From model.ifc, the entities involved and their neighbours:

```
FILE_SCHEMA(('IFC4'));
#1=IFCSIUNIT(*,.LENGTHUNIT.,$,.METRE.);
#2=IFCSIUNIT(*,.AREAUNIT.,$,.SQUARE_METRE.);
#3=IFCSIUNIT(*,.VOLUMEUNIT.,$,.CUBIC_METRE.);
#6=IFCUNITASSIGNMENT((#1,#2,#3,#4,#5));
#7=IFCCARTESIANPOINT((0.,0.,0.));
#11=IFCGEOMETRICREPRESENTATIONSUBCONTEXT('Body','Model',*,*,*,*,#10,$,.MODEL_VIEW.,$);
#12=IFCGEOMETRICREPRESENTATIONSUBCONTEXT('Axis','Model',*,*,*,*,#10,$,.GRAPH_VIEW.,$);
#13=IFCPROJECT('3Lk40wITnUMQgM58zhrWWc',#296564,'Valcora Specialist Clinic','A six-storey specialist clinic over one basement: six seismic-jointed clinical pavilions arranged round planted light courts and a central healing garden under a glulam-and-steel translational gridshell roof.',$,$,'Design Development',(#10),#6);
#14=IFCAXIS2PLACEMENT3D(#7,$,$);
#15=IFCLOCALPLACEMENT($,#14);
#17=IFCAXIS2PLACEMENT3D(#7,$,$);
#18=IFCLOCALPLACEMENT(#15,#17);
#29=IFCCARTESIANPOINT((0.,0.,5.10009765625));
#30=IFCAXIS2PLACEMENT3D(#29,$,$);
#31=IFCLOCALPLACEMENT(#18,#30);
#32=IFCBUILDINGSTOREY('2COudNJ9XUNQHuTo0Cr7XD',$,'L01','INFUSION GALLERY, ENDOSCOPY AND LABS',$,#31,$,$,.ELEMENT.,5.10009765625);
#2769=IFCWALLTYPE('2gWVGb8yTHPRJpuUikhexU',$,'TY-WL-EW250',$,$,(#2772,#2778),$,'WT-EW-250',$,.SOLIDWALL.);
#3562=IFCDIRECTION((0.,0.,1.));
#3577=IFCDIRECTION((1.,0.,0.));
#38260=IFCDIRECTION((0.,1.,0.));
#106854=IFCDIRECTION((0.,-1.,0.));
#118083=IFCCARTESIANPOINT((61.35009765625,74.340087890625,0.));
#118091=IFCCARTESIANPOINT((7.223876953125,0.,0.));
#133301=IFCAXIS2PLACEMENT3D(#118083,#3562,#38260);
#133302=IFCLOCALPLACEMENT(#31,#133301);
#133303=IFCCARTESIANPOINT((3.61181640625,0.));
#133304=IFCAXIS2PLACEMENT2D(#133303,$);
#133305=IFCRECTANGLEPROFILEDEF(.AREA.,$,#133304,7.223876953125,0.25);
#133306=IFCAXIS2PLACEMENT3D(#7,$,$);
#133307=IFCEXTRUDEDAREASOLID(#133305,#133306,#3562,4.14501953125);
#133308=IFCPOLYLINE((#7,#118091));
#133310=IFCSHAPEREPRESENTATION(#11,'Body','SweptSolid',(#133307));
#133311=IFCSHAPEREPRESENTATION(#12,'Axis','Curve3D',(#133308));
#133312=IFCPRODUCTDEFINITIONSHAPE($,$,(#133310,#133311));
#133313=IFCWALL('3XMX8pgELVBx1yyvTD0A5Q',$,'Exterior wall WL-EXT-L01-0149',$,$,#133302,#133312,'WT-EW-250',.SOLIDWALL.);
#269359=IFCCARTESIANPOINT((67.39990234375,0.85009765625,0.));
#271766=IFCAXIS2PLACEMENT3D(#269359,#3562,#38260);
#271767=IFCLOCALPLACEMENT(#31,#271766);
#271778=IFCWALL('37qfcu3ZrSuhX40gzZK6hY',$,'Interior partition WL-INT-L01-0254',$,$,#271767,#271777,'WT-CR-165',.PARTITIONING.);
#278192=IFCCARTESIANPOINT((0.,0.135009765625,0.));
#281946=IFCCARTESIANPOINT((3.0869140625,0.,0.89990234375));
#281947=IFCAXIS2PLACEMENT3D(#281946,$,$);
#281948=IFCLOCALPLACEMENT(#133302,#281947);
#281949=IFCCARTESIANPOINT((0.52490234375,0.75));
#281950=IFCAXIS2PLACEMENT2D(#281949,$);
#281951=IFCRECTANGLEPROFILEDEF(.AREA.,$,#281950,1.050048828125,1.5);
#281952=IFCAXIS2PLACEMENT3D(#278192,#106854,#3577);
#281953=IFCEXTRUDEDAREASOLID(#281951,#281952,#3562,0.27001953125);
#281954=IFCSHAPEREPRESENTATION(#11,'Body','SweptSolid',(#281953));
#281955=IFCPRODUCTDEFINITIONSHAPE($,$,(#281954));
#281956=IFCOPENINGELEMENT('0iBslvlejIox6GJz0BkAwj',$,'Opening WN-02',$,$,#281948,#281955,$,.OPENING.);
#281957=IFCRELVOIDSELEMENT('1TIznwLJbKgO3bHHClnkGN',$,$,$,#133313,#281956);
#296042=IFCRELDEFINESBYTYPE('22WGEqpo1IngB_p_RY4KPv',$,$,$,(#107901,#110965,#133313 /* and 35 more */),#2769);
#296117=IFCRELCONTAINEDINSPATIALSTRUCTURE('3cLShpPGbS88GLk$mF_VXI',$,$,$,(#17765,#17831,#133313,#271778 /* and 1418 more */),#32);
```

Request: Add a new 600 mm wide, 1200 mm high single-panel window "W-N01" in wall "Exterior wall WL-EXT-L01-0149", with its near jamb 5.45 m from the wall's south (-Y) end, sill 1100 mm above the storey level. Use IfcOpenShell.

```python
import numpy as np
import ifcopenshell
import ifcopenshell.api.feature
import ifcopenshell.api.geometry
import ifcopenshell.api.root
import ifcopenshell.api.spatial
import ifcopenshell.geom
import ifcopenshell.util.element
import ifcopenshell.util.placement
import ifcopenshell.util.representation
import ifcopenshell.util.shape
import ifcopenshell.util.unit

model = ifcopenshell.open("model.ifc")
unit_scale = ifcopenshell.util.unit.calculate_unit_scale(model)
settings = ifcopenshell.geom.settings()


def volume(element):
    """Net volume in cubic metres, openings subtracted."""
    shape = ifcopenshell.geom.create_shape(settings, element)
    return ifcopenshell.util.shape.get_volume(shape.geometry)


wall = model.by_guid("3XMX8pgELVBx1yyvTD0A5Q")
storey = ifcopenshell.util.element.get_container(wall, ifc_class="IfcBuildingStorey")
context = ifcopenshell.util.representation.get_context(model, "Model", "Body", "MODEL_VIEW")
before = volume(wall)

width, height, from_end, sill = 0.6, 1.2, 5.45, 1.1  # metres

# The wall runs along its own X axis, and the end named is its -X end.
wall_shape = ifcopenshell.geom.create_shape(settings, wall)
x, y, z = ifcopenshell.util.shape.get_vertices(wall_shape.geometry).T
start = x.min() + from_end
face, thickness = float(y.min()), float(y.max() - y.min())
wall_matrix = ifcopenshell.util.placement.get_local_placement(wall.ObjectPlacement)
level = ifcopenshell.util.placement.get_local_placement(storey.ObjectPlacement)[2, 3]


def in_wall(x, y):
    """Placement at x, y metres in the wall's axes, at sill height."""
    matrix = wall_matrix.copy()
    matrix[:, 3] = wall_matrix @ np.array([x / unit_scale, y / unit_scale, 0.0, 1.0])
    matrix[2, 3] = level + sill / unit_scale
    return matrix


# Opening: a box that overshoots both wall faces by 50 mm.
opening = ifcopenshell.api.root.create_entity(model, ifc_class="IfcOpeningElement", predefined_type="OPENING")
box = ifcopenshell.api.geometry.add_wall_representation(
    model, context=context, length=width, height=height, thickness=thickness + 0.1
)
ifcopenshell.api.geometry.assign_representation(model, product=opening, representation=box)
ifcopenshell.api.geometry.edit_object_placement(model, product=opening, matrix=in_wall(start, face - 0.05), is_si=False)
ifcopenshell.api.feature.add_feature(model, feature=opening, element=wall)

window = ifcopenshell.api.root.create_entity(model, ifc_class="IfcWindow", name="W-N01", predefined_type="WINDOW")
window.OverallWidth, window.OverallHeight = width / unit_scale, height / unit_scale
window.PartitioningType = "SINGLE_PANEL"
body = ifcopenshell.api.geometry.add_window_representation(
    model,
    context=context,
    overall_width=window.OverallWidth,
    overall_height=window.OverallHeight,
    partition_type="SINGLE_PANEL",
)
ifcopenshell.api.geometry.assign_representation(model, product=window, representation=body)
ifcopenshell.api.spatial.assign_container(model, products=[window], relating_structure=storey)
ifcopenshell.api.feature.add_filling(model, opening=opening, element=window)

# Centre the window in the wall's thickness.
ifcopenshell.api.geometry.edit_object_placement(model, product=window, matrix=in_wall(start, face), is_si=False)
window_shape = ifcopenshell.geom.create_shape(settings, window)
depth = ifcopenshell.util.shape.get_vertices(window_shape.geometry)[:, 1]
offset = face + thickness / 2 - (depth.min() + depth.max()) / 2
ifcopenshell.api.geometry.edit_object_placement(model, product=window, matrix=in_wall(start, offset), is_si=False)

after = volume(wall)

print(f"wall volume {before:.3f} -> {after:.3f} m3")

model.write("model_edited.ifc")
```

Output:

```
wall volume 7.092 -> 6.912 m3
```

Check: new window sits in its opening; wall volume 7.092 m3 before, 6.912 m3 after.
